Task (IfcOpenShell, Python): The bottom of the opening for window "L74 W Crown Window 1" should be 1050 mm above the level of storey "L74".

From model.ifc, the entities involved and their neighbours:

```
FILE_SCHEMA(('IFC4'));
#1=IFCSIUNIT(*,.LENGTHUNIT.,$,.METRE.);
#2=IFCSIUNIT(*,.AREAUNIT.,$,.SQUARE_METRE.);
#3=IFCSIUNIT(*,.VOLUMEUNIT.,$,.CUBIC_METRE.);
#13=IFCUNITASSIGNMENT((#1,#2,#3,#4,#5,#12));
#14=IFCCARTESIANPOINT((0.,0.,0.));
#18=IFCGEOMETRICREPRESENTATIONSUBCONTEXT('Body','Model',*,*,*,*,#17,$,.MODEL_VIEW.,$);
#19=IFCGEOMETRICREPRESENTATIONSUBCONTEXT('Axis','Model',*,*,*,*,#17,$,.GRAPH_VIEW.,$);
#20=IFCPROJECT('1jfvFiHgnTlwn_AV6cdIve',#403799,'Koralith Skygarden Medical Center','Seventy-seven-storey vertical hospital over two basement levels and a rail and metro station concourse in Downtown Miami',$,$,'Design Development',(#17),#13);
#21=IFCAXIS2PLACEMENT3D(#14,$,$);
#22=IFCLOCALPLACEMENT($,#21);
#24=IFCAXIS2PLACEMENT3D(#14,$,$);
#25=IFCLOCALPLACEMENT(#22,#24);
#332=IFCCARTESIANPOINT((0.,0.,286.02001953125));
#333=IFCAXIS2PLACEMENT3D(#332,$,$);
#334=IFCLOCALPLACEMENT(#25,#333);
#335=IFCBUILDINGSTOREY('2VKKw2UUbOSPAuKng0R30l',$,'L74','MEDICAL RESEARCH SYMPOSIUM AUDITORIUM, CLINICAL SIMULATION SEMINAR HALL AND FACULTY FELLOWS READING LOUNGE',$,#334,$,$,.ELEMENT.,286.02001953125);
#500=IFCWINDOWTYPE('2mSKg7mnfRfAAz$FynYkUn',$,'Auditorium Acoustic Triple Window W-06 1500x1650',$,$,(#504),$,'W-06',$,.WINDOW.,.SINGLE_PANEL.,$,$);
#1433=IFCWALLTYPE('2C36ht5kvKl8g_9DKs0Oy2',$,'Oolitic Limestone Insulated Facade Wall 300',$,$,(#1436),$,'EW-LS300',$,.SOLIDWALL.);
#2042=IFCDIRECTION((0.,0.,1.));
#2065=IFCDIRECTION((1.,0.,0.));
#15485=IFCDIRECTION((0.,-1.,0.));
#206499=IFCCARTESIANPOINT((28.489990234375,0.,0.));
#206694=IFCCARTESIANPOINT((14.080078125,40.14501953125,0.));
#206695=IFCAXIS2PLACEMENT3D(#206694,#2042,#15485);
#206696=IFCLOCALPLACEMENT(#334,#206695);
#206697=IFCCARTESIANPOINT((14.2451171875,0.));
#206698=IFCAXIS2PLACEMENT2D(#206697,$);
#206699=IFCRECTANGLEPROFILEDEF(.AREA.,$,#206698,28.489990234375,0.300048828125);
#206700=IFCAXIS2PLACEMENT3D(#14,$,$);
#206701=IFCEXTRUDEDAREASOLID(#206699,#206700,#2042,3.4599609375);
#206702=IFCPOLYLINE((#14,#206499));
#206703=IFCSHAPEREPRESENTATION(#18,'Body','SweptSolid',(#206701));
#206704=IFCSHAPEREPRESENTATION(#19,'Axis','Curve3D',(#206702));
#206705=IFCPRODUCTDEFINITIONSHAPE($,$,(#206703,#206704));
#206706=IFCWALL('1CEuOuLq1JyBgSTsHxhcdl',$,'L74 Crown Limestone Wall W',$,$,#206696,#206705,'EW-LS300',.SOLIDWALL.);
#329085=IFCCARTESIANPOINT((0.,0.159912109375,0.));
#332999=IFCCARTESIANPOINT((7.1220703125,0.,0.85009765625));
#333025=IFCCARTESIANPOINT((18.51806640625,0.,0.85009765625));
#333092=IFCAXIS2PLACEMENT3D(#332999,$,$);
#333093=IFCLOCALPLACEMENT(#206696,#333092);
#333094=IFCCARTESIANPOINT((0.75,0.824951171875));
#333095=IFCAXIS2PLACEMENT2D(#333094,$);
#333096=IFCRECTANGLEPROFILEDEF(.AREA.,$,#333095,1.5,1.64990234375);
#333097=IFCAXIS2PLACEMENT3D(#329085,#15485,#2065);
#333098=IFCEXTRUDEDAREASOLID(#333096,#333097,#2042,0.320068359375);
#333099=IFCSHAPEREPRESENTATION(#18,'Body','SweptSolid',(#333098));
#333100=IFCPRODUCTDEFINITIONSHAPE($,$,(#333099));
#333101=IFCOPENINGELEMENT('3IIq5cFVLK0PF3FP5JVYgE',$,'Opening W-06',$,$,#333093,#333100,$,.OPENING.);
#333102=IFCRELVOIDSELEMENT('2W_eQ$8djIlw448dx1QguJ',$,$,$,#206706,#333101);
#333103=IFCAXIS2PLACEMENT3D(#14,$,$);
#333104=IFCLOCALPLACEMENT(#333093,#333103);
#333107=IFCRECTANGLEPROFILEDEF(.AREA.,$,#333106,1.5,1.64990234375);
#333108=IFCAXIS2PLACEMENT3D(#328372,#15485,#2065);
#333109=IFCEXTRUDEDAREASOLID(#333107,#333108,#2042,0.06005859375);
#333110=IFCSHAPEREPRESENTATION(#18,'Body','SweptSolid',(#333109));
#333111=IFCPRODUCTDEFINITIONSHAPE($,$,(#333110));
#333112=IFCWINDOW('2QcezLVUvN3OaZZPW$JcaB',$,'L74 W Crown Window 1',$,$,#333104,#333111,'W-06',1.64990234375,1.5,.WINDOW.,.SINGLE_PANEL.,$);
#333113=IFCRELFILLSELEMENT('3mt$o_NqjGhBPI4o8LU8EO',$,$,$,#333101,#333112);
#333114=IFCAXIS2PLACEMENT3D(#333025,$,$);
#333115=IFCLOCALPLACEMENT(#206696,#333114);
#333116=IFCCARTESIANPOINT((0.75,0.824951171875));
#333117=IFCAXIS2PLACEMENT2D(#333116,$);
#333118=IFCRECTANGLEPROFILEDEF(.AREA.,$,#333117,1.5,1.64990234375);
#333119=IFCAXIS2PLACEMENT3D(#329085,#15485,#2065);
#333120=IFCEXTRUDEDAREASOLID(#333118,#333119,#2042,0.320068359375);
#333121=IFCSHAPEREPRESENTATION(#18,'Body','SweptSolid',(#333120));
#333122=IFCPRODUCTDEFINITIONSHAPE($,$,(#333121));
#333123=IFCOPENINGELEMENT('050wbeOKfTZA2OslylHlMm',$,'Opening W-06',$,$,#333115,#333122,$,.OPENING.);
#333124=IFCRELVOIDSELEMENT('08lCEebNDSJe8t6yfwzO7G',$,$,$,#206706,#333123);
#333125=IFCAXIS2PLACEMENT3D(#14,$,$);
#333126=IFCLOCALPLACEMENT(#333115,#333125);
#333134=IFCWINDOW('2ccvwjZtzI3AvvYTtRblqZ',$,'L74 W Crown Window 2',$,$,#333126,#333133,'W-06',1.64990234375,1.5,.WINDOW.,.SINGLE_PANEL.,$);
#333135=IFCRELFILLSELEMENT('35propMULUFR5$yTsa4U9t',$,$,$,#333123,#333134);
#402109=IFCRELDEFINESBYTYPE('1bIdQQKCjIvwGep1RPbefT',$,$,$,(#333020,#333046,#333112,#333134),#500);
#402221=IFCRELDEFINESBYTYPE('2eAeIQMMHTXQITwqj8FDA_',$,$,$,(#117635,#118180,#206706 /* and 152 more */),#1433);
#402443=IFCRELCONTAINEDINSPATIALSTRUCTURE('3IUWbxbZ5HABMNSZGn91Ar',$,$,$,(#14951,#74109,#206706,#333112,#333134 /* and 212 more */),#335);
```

```python
import numpy as np
import ifcopenshell
import ifcopenshell.api.geometry
import ifcopenshell.geom
import ifcopenshell.util.element
import ifcopenshell.util.placement
import ifcopenshell.util.shape
import ifcopenshell.util.unit

model = ifcopenshell.open("model.ifc")
unit_scale = ifcopenshell.util.unit.calculate_unit_scale(model)

window = model.by_id(333112)
opening = window.FillsVoids[0].RelatingOpeningElement
storey = ifcopenshell.util.element.get_container(window, ifc_class="IfcBuildingStorey")
level = ifcopenshell.util.placement.get_local_placement(storey.ObjectPlacement)[2, 3]

# The opening's origin need not be at the sill, so measure its lowest point.
shape = ifcopenshell.geom.create_shape(ifcopenshell.geom.settings(), opening)
bottom = ifcopenshell.util.shape.get_shape_bottom_elevation(shape, shape.geometry) / unit_scale
dz = level + 1.05 / unit_scale - bottom

shift = np.array([0.0, 0.0, dz])
# The window is placed relative to its opening, so it follows when the opening moves.
matrix = ifcopenshell.util.placement.get_local_placement(opening.ObjectPlacement)
matrix[:3, 3] += shift
ifcopenshell.api.geometry.edit_object_placement(
    model, product=opening, matrix=matrix, is_si=False, should_transform_children=True
)

print(f"moved by {dz * unit_scale:+.3f} m")

model.write("model_edited.ifc")
```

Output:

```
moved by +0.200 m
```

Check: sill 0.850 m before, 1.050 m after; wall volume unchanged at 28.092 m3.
